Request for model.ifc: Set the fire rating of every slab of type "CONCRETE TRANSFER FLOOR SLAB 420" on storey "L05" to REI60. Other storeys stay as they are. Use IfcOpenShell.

First a look at what the model holds.

```python
import ifcopenshell
import ifcopenshell.util.element

model = ifcopenshell.open("model.ifc")
print(model.schema)
storey = next(s for s in model.by_type("IfcBuildingStorey") if s.Name == "L05")
slabs = [e for e in ifcopenshell.util.element.get_decomposition(storey) if e.is_a("IfcSlab")]
seen = {}
for e in slabs:
    element_type = ifcopenshell.util.element.get_type(e)
    key = (element_type.Name if element_type != e and element_type else None, ifcopenshell.util.element.get_pset(e, "Pset_SlabCommon", "FireRating"))
    seen[key] = seen.get(key, 0) + 1
for (name, value), count in sorted(seen.items(), key=str):
    print(count, "x", name, "|", value)
```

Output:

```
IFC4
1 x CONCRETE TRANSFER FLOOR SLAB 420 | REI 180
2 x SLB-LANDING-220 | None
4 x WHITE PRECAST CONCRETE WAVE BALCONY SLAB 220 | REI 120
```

```python
import ifcopenshell
import ifcopenshell.api.pset
import ifcopenshell.util.element

model = ifcopenshell.open("model.ifc")

storey = next(s for s in model.by_type("IfcBuildingStorey") if s.Name == "L05")
slabs = [e for e in ifcopenshell.util.element.get_decomposition(storey) if e.is_a("IfcSlab")]

count = 0
for e in slabs:
    element_type = ifcopenshell.util.element.get_type(e)
    if element_type in (None, e) or element_type.Name != "CONCRETE TRANSFER FLOOR SLAB 420":
        continue
    found = ifcopenshell.util.element.get_pset(e, "Pset_SlabCommon", should_inherit=False)
    if found:
        pset = model.by_id(found["id"])
        if len(ifcopenshell.util.element.get_elements_by_pset(pset)) > 1:
            pset = ifcopenshell.api.pset.unshare_pset(model, products=[e], pset=pset)[0]
    else:
        pset = ifcopenshell.api.pset.add_pset(model, product=e, name="Pset_SlabCommon")
    ifcopenshell.api.pset.edit_pset(model, pset=pset, properties={"FireRating": "REI60"})
    count += 1

print(count, "slabs updated")

model.write("model_edited.ifc")
```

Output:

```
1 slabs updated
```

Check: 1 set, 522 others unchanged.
